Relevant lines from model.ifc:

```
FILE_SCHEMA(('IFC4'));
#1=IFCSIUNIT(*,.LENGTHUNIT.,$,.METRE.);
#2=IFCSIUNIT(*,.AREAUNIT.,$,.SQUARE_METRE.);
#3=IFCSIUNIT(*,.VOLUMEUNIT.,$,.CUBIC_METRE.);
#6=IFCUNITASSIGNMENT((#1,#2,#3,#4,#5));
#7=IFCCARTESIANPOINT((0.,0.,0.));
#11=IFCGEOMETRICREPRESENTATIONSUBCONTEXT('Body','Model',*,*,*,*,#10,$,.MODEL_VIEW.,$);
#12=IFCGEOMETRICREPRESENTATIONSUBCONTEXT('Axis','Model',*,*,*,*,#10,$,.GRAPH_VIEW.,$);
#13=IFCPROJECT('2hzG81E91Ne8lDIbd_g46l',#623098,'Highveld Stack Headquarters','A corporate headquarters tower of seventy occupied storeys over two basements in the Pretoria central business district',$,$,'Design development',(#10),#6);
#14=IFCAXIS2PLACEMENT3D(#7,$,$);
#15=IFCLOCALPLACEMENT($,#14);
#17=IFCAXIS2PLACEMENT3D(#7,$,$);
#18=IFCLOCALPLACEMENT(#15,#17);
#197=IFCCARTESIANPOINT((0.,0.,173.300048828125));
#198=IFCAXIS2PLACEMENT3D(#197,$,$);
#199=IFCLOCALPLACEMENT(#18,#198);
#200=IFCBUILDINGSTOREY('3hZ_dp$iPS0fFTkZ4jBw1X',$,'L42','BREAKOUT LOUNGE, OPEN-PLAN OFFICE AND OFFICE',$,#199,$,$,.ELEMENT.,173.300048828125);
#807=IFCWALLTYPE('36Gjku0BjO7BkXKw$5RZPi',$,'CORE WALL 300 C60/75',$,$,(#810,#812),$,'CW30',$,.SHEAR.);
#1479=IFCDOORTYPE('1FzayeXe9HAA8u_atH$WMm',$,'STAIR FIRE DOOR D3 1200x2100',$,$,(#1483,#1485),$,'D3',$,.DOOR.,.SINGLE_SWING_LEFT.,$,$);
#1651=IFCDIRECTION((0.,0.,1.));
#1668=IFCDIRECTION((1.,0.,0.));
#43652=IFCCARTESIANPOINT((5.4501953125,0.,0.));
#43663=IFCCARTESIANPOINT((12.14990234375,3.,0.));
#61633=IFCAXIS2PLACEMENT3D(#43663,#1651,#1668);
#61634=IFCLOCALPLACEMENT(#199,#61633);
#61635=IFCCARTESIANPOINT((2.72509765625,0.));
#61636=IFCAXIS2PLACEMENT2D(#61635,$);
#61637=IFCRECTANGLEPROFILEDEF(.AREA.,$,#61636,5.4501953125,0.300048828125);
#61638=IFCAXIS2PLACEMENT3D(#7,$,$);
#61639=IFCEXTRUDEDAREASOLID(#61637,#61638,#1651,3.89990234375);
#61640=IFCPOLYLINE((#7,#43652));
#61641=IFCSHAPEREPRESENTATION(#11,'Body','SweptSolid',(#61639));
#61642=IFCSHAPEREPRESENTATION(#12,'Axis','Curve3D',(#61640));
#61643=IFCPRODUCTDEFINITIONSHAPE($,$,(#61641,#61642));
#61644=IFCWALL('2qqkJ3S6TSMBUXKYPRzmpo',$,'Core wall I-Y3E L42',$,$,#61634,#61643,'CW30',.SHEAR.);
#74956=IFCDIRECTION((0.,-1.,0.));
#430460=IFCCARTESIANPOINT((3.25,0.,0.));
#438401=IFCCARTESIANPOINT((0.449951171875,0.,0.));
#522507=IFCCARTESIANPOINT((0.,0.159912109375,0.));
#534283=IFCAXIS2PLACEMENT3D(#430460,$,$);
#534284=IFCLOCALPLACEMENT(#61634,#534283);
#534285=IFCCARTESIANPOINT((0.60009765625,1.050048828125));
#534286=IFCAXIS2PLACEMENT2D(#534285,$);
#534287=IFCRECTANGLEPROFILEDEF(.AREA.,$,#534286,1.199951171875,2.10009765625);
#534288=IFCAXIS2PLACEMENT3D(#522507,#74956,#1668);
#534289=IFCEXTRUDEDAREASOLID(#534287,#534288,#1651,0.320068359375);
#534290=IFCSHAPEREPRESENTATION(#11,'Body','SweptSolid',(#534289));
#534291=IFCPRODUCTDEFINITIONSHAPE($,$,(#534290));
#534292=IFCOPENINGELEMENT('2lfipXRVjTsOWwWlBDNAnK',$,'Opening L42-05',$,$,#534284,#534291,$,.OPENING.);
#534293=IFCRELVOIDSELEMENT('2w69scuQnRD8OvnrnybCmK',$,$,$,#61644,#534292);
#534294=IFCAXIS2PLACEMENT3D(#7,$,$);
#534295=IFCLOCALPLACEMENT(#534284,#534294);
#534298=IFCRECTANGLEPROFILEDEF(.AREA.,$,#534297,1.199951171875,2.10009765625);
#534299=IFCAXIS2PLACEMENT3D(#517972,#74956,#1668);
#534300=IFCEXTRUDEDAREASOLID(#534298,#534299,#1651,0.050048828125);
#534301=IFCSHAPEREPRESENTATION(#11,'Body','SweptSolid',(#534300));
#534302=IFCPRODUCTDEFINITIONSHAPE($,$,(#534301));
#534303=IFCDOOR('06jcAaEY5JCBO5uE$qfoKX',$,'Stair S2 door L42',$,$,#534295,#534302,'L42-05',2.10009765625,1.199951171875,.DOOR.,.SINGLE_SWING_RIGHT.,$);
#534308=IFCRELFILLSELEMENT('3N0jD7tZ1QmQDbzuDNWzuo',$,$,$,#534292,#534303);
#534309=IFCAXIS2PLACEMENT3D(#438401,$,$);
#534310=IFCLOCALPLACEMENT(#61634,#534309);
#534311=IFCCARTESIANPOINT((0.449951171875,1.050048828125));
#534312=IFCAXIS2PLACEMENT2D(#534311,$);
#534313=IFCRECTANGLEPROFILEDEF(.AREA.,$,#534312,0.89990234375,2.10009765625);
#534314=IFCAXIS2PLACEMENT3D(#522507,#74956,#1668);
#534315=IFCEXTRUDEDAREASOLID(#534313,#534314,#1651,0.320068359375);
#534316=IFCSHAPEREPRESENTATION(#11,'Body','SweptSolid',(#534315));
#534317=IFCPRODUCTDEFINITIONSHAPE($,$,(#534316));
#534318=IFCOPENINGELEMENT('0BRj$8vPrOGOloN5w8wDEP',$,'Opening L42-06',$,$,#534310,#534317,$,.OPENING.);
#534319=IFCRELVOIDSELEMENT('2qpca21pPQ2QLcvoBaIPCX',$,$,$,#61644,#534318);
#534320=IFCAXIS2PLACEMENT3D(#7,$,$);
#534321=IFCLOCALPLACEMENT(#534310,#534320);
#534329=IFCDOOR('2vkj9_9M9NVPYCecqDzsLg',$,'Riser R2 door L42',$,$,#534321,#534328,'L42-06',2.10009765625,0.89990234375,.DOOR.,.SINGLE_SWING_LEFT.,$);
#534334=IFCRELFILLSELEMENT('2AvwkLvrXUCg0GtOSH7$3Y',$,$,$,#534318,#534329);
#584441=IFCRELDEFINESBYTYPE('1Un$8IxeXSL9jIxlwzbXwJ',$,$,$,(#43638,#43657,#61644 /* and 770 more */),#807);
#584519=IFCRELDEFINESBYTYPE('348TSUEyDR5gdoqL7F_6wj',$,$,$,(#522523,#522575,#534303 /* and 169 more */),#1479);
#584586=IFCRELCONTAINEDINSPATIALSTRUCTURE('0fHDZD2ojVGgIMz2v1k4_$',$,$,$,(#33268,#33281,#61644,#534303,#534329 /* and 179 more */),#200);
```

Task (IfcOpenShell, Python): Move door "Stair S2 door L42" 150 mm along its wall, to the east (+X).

```python
import ifcopenshell
import ifcopenshell.api.geometry
import ifcopenshell.util.placement
import ifcopenshell.util.unit

model = ifcopenshell.open("model.ifc")
unit_scale = ifcopenshell.util.unit.calculate_unit_scale(model)

door = model.by_id(534303)
opening = door.FillsVoids[0].RelatingOpeningElement
wall = opening.VoidsElements[0].RelatingBuildingElement

wall_matrix = ifcopenshell.util.placement.get_local_placement(wall.ObjectPlacement)
shift = wall_matrix[:3, 0] * 0.15 / unit_scale
before = ifcopenshell.util.placement.get_local_placement(door.ObjectPlacement)[:3, 3].copy()

# The door is placed relative to its opening, so it follows when the opening moves.
matrix = ifcopenshell.util.placement.get_local_placement(opening.ObjectPlacement)
matrix[:3, 3] += shift
ifcopenshell.api.geometry.edit_object_placement(
    model, product=opening, matrix=matrix, is_si=False, should_transform_children=True
)

after = ifcopenshell.util.placement.get_local_placement(door.ObjectPlacement)[:3, 3]
print("door moved by", (after - before).round(3) + 0.0)

model.write("model_rev.ifc")
```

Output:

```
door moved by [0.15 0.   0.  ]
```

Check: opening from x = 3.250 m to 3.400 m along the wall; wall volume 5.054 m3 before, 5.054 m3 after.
